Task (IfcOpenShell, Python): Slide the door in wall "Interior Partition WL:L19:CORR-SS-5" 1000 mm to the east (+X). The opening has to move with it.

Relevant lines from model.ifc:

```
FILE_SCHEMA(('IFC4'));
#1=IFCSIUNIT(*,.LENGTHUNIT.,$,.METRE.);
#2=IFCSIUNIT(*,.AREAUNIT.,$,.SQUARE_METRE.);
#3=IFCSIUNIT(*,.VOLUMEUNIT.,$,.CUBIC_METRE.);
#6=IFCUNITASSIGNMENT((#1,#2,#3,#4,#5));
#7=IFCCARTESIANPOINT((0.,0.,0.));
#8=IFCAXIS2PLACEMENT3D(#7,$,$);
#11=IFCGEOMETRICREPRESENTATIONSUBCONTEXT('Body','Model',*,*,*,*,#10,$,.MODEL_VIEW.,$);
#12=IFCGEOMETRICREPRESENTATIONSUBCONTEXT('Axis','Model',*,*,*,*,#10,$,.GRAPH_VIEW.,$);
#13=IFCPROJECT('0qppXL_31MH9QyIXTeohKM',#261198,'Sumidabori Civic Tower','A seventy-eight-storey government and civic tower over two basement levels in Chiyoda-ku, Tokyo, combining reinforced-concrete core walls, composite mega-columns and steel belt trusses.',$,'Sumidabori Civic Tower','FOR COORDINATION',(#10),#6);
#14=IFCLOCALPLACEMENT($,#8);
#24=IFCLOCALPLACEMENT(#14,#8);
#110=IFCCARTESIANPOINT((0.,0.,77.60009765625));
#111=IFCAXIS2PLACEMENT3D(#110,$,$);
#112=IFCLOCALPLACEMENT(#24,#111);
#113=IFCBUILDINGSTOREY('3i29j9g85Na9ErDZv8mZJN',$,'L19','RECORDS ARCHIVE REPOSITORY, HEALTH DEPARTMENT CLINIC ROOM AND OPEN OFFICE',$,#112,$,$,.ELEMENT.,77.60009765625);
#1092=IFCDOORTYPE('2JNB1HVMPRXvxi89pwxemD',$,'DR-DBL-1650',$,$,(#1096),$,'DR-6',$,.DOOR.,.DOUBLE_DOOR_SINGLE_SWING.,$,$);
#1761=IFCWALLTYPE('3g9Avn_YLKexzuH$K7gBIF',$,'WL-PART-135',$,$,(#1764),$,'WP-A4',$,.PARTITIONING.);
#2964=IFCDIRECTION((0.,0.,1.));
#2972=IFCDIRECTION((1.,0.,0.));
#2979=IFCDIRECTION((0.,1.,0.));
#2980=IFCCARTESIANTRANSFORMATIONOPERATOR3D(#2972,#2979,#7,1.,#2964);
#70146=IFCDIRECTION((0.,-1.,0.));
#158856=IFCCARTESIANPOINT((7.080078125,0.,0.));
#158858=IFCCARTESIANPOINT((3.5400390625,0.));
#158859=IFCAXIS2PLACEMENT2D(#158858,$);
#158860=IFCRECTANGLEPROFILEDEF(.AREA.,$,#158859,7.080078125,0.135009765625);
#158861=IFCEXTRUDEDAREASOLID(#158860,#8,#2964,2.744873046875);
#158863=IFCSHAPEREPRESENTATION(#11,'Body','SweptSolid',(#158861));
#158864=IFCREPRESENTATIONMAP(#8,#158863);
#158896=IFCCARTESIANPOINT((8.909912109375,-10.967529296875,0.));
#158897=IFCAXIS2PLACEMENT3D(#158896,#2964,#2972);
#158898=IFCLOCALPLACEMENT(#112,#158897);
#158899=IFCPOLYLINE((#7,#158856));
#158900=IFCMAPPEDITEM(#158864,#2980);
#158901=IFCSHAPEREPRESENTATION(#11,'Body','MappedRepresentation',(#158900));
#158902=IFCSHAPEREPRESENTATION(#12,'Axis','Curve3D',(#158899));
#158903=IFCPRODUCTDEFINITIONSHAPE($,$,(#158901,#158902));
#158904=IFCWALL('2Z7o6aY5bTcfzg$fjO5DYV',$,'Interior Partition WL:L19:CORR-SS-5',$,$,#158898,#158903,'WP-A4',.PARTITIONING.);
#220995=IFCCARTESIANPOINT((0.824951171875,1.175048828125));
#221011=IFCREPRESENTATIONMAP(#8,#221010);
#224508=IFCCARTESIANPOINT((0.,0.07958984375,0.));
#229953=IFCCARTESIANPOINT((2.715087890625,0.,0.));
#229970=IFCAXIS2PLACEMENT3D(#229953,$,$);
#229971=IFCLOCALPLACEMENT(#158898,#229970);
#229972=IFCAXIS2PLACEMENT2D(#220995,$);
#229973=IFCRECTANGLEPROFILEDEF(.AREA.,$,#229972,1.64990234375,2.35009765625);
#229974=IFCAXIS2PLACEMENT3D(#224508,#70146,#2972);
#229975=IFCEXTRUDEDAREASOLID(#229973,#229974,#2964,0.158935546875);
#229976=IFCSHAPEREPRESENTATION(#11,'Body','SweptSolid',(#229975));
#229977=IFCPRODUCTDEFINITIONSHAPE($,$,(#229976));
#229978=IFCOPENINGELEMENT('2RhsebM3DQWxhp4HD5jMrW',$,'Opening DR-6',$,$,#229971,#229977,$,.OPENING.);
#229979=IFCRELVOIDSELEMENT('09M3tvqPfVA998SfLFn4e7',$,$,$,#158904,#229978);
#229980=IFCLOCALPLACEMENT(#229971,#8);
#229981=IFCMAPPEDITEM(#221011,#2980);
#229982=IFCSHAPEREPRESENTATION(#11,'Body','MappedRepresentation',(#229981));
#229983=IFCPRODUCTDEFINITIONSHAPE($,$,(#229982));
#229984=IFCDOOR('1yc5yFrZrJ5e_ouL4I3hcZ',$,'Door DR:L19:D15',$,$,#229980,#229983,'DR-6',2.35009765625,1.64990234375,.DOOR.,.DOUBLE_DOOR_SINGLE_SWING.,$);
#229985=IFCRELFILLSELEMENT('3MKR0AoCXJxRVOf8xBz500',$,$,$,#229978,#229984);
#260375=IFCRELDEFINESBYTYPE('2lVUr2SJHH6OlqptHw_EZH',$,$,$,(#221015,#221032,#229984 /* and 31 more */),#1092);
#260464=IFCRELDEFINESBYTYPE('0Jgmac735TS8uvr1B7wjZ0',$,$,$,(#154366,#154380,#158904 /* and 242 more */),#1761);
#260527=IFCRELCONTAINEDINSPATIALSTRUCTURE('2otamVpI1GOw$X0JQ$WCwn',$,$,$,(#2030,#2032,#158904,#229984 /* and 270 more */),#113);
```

```python
import ifcopenshell
import ifcopenshell.api.geometry
import ifcopenshell.util.placement
import ifcopenshell.util.unit

model = ifcopenshell.open("model.ifc")
unit_scale = ifcopenshell.util.unit.calculate_unit_scale(model)

door = model.by_guid("1yc5yFrZrJ5e_ouL4I3hcZ")
opening = door.FillsVoids[0].RelatingOpeningElement
wall = opening.VoidsElements[0].RelatingBuildingElement

wall_matrix = ifcopenshell.util.placement.get_local_placement(wall.ObjectPlacement)
shift = wall_matrix[:3, 0] * 1 / unit_scale
before = ifcopenshell.util.placement.get_local_placement(door.ObjectPlacement)[:3, 3].copy()

# The door is placed relative to its opening, so it follows when the opening moves.
matrix = ifcopenshell.util.placement.get_local_placement(opening.ObjectPlacement)
matrix[:3, 3] += shift
ifcopenshell.api.geometry.edit_object_placement(
    model, product=opening, matrix=matrix, is_si=False, should_transform_children=True
)

after = ifcopenshell.util.placement.get_local_placement(door.ObjectPlacement)[:3, 3]
print("door moved by", (after - before).round(3) + 0.0)

model.write("model_updated.ifc")
```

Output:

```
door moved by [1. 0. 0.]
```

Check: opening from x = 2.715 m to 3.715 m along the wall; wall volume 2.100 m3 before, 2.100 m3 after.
